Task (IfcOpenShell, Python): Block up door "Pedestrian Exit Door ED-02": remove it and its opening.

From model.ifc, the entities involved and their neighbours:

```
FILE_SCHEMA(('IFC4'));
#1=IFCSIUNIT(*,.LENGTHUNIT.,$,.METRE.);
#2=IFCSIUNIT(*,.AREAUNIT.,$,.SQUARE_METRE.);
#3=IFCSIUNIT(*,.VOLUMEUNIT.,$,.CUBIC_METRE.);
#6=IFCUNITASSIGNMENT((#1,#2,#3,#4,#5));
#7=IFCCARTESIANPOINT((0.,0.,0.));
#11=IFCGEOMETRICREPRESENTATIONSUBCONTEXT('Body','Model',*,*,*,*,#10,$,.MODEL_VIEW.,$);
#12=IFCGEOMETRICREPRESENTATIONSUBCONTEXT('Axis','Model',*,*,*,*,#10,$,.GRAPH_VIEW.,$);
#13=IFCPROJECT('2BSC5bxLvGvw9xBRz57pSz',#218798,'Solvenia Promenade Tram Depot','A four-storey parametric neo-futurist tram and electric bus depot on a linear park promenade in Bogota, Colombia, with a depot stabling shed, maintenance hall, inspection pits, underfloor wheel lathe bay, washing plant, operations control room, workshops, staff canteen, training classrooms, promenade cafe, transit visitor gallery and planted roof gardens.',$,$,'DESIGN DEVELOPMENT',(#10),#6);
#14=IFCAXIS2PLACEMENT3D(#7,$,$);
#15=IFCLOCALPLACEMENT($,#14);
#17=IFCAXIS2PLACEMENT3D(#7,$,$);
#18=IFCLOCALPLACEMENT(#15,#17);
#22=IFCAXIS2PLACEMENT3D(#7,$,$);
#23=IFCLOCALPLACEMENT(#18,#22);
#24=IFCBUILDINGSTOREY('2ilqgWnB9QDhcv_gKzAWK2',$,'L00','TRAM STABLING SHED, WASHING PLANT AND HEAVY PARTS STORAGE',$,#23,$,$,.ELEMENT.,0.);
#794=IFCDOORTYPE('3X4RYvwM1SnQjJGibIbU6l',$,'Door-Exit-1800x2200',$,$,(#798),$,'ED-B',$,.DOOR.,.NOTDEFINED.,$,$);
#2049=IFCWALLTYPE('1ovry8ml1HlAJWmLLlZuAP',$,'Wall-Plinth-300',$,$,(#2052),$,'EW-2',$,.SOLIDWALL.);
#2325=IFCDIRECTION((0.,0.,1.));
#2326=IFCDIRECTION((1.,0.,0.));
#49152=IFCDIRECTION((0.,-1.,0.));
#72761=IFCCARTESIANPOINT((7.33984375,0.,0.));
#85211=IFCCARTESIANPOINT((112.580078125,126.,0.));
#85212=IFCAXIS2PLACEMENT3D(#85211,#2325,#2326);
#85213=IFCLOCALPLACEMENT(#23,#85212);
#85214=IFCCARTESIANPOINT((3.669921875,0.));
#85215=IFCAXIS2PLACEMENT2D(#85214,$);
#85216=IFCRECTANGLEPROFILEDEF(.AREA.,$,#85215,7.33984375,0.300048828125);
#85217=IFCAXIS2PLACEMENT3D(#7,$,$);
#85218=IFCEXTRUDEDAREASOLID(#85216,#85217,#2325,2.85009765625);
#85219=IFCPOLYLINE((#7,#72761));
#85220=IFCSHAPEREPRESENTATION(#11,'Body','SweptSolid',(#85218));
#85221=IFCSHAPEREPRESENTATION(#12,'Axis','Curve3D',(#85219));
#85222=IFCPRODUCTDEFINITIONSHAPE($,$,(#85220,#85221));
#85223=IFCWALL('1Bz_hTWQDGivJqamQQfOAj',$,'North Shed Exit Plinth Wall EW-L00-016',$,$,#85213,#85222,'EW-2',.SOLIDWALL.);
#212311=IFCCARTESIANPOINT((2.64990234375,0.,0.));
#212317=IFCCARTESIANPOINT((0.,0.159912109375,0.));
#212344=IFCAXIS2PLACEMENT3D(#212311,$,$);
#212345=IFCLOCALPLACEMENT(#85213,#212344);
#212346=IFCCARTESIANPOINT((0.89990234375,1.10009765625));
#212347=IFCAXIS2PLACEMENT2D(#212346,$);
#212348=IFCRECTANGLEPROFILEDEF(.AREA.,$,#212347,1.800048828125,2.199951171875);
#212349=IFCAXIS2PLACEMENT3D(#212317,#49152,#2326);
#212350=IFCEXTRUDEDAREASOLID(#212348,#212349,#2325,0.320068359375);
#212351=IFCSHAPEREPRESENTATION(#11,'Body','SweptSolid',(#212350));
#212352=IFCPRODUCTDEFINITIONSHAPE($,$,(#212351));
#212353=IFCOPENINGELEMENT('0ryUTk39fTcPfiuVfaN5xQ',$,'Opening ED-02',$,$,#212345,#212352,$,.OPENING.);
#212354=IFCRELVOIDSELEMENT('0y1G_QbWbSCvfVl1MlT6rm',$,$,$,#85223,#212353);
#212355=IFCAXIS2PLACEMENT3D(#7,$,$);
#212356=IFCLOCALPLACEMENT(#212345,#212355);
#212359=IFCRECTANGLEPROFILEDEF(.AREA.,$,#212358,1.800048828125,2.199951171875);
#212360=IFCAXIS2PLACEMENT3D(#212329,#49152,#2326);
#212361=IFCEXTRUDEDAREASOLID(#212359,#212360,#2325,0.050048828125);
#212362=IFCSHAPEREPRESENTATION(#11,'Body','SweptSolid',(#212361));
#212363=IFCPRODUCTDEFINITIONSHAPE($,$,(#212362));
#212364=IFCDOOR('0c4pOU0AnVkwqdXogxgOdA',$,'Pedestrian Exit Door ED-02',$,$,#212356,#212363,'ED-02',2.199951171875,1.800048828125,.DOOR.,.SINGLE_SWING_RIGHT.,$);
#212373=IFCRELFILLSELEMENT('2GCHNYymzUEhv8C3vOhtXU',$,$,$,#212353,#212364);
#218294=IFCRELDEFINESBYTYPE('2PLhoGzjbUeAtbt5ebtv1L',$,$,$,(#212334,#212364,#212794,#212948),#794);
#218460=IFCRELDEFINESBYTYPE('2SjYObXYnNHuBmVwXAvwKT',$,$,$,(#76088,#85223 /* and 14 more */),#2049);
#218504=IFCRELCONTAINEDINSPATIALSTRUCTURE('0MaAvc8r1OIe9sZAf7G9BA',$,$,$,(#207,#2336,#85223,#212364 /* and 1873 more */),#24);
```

```python
import ifcopenshell
import ifcopenshell.api.feature
import ifcopenshell.api.root
import ifcopenshell.geom
import ifcopenshell.util.shape

model = ifcopenshell.open("model.ifc")
settings = ifcopenshell.geom.settings()


def volume(element):
    """Net volume in cubic metres, openings subtracted."""
    shape = ifcopenshell.geom.create_shape(settings, element)
    return ifcopenshell.util.shape.get_volume(shape.geometry)


door = model.by_guid("0c4pOU0AnVkwqdXogxgOdA")
opening = door.FillsVoids[0].RelatingOpeningElement
wall = opening.VoidsElements[0].RelatingBuildingElement
before = volume(wall)

ifcopenshell.api.root.remove_product(model, product=door)
ifcopenshell.api.feature.remove_feature(model, feature=opening)

after = volume(wall)

print(f"wall volume {before:.3f} -> {after:.3f} m3")

model.write("model_updated.ifc")
```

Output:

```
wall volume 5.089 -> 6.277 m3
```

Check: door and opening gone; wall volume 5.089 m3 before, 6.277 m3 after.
